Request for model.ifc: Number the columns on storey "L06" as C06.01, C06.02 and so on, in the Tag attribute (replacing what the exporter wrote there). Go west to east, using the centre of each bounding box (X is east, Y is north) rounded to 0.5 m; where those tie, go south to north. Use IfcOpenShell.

First a look at what the model holds.

```python
import ifcopenshell
import ifcopenshell.util.element
import ifcopenshell.util.placement

model = ifcopenshell.open("model.ifc")
print(model.schema)
storey = next(s for s in model.by_type("IfcBuildingStorey") if s.Name == "L06")
columns = [e for e in ifcopenshell.util.element.get_decomposition(storey) if e.is_a("IfcColumn")]
for e in sorted(columns, key=lambda e: e.id()):
    origin = ifcopenshell.util.placement.get_local_placement(e.ObjectPlacement)[:3, 3]
    print(e.id(), e.Tag, e.Name, origin.round(2) + 0.0, sep=" | ")
```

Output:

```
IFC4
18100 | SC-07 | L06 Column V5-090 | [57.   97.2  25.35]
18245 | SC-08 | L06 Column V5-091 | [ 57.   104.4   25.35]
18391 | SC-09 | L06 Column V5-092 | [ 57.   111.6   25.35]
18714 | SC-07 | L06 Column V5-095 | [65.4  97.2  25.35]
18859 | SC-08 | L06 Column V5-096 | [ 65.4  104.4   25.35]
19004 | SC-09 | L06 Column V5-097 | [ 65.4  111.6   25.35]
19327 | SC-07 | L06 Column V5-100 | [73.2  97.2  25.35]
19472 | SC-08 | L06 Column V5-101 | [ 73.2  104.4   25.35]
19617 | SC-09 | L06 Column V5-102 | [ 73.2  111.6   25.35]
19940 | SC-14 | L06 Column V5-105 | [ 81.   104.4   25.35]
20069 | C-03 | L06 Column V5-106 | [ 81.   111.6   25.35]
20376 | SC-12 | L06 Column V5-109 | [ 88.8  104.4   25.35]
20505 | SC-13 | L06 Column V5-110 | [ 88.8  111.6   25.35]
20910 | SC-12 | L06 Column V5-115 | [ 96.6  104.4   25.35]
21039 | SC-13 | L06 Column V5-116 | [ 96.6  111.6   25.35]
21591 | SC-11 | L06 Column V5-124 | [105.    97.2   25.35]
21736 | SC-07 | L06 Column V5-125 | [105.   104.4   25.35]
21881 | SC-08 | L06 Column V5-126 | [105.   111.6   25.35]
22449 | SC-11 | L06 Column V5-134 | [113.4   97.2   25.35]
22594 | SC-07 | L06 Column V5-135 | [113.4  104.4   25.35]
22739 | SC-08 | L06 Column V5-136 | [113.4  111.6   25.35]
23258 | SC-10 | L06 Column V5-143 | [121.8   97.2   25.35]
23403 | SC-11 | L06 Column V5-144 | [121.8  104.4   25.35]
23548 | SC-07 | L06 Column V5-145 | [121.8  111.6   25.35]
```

```python
import ifcopenshell
import ifcopenshell.geom
import ifcopenshell.util.element
import ifcopenshell.util.shape

model = ifcopenshell.open("model.ifc")
settings = ifcopenshell.geom.settings()
settings.set("use-world-coords", True)


def centre(element):
    shape = ifcopenshell.geom.create_shape(settings, element)
    return ifcopenshell.util.shape.get_bbox_centroid(shape.geometry)


storey = next(s for s in model.by_type("IfcBuildingStorey") if s.Name == "L06")
columns = [e for e in ifcopenshell.util.element.get_decomposition(storey) if e.is_a("IfcColumn")]

# Insertion points can sit at a corner or the storey origin, so sort by the geometry (in metres).
centres = {e: centre(e) for e in columns}
columns.sort(key=lambda e: (round(centres[e][0] / 0.5), centres[e][1]))

for i, e in enumerate(columns, start=1):
    number = f"C06.{i:02d}"
    e.Tag = number
    print(e.id(), number)

model.write("model_rev.ifc")
```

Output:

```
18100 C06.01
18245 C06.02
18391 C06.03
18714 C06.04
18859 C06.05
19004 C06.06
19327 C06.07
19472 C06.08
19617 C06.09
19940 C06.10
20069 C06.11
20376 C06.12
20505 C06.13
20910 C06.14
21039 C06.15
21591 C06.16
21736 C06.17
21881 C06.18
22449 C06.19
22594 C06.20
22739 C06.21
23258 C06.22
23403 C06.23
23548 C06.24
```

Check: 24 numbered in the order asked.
